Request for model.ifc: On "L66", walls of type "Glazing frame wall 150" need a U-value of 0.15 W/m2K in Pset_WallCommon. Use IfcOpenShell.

First a look at what the model holds.

```python
import ifcopenshell
import ifcopenshell.util.element

model = ifcopenshell.open("model.ifc")
print(model.schema)
storey = next(s for s in model.by_type("IfcBuildingStorey") if s.Name == "L66")
walls = [e for e in ifcopenshell.util.element.get_decomposition(storey) if e.is_a("IfcWall")]
seen = {}
for e in walls:
    element_type = ifcopenshell.util.element.get_type(e)
    key = (element_type.Name if element_type != e and element_type else None, ifcopenshell.util.element.get_pset(e, "Pset_WallCommon", "ThermalTransmittance"))
    seen[key] = seen.get(key, 0) + 1
for (name, value), count in sorted(seen.items(), key=str):
    print(count, "x", name, "|", value)
```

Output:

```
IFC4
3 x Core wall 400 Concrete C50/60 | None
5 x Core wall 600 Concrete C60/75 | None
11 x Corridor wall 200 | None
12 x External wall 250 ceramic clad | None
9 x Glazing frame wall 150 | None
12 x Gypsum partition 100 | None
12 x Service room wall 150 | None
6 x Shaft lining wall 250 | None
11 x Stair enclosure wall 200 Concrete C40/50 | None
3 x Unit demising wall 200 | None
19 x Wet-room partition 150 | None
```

```python
import ifcopenshell
import ifcopenshell.api.pset
import ifcopenshell.util.element

model = ifcopenshell.open("model.ifc")

storey = next(s for s in model.by_type("IfcBuildingStorey") if s.Name == "L66")
walls = [e for e in ifcopenshell.util.element.get_decomposition(storey) if e.is_a("IfcWall")]

count = 0
for e in walls:
    element_type = ifcopenshell.util.element.get_type(e)
    if element_type in (None, e) or element_type.Name != "Glazing frame wall 150":
        continue
    found = ifcopenshell.util.element.get_pset(e, "Pset_WallCommon", should_inherit=False)
    if found:
        pset = model.by_id(found["id"])
        if len(ifcopenshell.util.element.get_elements_by_pset(pset)) > 1:
            pset = ifcopenshell.api.pset.unshare_pset(model, products=[e], pset=pset)[0]
    else:
        pset = ifcopenshell.api.pset.add_pset(model, product=e, name="Pset_WallCommon")
    ifcopenshell.api.pset.edit_pset(model, pset=pset, properties={"ThermalTransmittance": 0.15})
    count += 1

print(count, "walls updated")

model.write("model-out.ifc")
```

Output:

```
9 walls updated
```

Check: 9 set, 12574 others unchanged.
